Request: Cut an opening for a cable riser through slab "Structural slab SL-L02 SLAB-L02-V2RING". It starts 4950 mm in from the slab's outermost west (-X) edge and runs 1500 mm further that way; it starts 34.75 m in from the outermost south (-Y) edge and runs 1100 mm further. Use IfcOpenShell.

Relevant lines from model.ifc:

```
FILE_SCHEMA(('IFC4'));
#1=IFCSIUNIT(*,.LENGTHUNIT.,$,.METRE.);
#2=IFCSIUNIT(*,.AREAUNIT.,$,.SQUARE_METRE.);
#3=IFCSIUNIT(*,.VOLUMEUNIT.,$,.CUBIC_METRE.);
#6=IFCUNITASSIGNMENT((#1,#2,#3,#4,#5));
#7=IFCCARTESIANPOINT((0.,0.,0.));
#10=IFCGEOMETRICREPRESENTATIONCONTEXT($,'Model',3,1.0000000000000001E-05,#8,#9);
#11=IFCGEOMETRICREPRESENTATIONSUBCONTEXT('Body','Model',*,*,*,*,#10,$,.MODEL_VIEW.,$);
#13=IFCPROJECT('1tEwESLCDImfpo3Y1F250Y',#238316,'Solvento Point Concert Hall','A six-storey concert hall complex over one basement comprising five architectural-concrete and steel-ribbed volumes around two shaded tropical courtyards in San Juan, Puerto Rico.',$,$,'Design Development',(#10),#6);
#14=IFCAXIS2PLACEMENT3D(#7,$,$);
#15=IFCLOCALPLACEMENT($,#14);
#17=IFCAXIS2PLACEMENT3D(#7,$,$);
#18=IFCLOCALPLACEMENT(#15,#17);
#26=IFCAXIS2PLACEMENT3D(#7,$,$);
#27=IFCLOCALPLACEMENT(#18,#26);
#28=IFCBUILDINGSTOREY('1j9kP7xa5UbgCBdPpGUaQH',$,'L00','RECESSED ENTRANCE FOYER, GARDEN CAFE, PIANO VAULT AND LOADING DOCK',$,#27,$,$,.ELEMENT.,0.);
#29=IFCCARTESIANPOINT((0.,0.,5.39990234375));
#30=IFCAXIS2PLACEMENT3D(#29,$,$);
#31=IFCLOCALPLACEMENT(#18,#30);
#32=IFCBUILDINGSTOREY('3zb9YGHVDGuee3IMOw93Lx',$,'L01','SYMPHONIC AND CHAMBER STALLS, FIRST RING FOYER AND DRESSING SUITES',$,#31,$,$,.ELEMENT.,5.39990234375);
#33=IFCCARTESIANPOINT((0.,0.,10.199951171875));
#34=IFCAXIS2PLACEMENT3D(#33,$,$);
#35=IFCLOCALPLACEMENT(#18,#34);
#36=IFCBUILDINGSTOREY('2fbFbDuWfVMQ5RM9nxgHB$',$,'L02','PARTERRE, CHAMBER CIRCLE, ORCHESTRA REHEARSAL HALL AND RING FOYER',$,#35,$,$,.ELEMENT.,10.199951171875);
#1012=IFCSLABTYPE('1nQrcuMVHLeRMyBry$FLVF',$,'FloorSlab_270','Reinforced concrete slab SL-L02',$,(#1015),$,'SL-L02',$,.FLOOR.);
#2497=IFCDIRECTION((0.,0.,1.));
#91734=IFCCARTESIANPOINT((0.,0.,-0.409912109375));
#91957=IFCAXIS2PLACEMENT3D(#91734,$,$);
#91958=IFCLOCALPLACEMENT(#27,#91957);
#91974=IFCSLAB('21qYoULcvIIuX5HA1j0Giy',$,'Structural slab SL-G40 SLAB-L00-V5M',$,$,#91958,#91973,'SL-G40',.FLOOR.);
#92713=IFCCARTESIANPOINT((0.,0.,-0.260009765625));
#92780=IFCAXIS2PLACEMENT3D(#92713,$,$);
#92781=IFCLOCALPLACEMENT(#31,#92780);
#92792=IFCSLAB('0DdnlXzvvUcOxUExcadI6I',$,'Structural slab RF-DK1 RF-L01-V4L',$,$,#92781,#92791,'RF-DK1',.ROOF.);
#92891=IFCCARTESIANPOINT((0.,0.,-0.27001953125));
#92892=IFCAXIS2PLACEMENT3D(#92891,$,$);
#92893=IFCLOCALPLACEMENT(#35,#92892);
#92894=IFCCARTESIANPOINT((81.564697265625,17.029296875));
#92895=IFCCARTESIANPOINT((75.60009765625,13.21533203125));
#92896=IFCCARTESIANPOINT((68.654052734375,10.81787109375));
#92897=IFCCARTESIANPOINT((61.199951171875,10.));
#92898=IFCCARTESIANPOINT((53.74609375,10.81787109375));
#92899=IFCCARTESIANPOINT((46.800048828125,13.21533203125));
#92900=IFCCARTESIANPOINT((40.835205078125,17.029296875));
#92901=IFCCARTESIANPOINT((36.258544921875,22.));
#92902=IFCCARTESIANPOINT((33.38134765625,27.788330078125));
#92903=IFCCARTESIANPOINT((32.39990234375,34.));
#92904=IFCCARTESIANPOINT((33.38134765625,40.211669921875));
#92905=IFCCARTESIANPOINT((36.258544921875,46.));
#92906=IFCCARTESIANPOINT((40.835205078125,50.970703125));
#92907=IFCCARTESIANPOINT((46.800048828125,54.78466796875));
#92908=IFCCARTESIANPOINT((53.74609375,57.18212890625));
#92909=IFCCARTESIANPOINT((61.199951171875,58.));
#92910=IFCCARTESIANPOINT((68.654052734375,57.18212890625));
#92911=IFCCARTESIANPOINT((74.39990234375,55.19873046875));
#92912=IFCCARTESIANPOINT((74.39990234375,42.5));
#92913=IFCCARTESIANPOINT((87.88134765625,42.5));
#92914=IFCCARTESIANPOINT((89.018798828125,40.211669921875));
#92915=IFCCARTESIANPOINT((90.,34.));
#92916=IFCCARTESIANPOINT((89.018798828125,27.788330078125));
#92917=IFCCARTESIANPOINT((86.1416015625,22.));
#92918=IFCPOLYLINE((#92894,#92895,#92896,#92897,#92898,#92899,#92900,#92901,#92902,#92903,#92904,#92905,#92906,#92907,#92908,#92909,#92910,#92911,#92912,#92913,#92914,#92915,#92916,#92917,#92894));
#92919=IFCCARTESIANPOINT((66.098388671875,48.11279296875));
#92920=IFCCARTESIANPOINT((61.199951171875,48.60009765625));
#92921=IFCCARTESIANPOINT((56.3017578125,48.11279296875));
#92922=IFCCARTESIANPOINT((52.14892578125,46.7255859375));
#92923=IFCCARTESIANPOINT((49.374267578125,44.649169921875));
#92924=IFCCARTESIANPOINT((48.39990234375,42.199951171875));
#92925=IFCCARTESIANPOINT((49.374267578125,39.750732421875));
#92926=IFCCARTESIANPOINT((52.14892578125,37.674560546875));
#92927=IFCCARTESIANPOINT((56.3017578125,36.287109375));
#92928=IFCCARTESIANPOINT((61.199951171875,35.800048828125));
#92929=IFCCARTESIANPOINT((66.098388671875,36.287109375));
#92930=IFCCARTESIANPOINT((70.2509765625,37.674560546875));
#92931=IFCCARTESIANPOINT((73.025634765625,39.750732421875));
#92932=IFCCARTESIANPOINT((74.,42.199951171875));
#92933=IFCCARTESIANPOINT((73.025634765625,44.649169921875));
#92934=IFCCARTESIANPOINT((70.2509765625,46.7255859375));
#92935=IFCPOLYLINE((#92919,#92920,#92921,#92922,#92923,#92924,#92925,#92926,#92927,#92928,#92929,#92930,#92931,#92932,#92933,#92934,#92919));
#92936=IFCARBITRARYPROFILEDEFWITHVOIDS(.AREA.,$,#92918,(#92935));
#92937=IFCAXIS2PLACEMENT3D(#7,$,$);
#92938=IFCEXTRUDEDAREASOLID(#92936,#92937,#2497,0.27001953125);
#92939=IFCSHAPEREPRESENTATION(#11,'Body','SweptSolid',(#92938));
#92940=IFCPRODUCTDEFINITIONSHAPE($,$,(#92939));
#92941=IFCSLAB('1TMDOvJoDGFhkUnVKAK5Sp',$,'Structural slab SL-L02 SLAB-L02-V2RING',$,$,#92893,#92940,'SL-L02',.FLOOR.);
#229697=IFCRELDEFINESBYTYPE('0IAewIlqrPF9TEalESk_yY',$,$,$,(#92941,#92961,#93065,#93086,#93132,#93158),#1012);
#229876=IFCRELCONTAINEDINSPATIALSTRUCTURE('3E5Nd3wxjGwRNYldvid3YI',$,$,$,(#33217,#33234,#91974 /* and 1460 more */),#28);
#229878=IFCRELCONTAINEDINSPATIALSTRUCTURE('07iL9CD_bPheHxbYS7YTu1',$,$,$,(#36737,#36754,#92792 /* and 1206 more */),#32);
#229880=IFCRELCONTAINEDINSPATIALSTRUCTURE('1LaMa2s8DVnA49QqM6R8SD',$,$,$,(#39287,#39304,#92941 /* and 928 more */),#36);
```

```python
import numpy as np
import ifcopenshell
import ifcopenshell.api.feature
import ifcopenshell.api.geometry
import ifcopenshell.api.root
import ifcopenshell.geom
import ifcopenshell.util.placement
import ifcopenshell.util.representation
import ifcopenshell.util.shape
import ifcopenshell.util.unit

model = ifcopenshell.open("model.ifc")
unit_scale = ifcopenshell.util.unit.calculate_unit_scale(model)
settings = ifcopenshell.geom.settings()


def volume(element):
    """Net volume in cubic metres, openings subtracted."""
    shape = ifcopenshell.geom.create_shape(settings, element)
    return ifcopenshell.util.shape.get_volume(shape.geometry)


slab = model.by_id(92941)
before = volume(slab)

# Extent in the slab's own axes, in metres. The edges named are its -X and -Y sides.
slab_shape = ifcopenshell.geom.create_shape(settings, slab)
vertices = ifcopenshell.util.shape.get_vertices(slab_shape.geometry)
x_min, y_min, bottom = vertices.min(axis=0)
top = vertices[:, 2].max()

opening = ifcopenshell.api.root.create_entity(model, ifc_class="IfcOpeningElement", name="Cable riser opening", predefined_type="OPENING")
context = ifcopenshell.util.representation.get_context(model, "Model", "Body", "MODEL_VIEW")
width, depth = 1.5, 1.1
outline = [(0.0, 0.0), (width, 0.0), (width, depth), (0.0, depth), (0.0, 0.0)]
# Overshoot both faces by 50 mm so the cut is clean.
shape = ifcopenshell.api.geometry.add_slab_representation(
    model, context=context, depth=top - bottom + 0.1, polyline=outline
)
ifcopenshell.api.geometry.assign_representation(model, product=opening, representation=shape)

matrix = ifcopenshell.util.placement.get_local_placement(slab.ObjectPlacement)
matrix[:, 3] = matrix @ np.append(np.array([x_min + 4.95, y_min + 34.75, bottom - 0.05]) / unit_scale, 1.0)
ifcopenshell.api.geometry.edit_object_placement(model, product=opening, matrix=matrix, is_si=False)
ifcopenshell.api.feature.add_feature(model, feature=opening, element=slab)

after = volume(slab)

print(f"slab volume {before:.3f} -> {after:.3f} m3")

model.write("model_rev.ifc")
```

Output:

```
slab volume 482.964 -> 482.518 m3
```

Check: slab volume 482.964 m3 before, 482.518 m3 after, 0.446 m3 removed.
